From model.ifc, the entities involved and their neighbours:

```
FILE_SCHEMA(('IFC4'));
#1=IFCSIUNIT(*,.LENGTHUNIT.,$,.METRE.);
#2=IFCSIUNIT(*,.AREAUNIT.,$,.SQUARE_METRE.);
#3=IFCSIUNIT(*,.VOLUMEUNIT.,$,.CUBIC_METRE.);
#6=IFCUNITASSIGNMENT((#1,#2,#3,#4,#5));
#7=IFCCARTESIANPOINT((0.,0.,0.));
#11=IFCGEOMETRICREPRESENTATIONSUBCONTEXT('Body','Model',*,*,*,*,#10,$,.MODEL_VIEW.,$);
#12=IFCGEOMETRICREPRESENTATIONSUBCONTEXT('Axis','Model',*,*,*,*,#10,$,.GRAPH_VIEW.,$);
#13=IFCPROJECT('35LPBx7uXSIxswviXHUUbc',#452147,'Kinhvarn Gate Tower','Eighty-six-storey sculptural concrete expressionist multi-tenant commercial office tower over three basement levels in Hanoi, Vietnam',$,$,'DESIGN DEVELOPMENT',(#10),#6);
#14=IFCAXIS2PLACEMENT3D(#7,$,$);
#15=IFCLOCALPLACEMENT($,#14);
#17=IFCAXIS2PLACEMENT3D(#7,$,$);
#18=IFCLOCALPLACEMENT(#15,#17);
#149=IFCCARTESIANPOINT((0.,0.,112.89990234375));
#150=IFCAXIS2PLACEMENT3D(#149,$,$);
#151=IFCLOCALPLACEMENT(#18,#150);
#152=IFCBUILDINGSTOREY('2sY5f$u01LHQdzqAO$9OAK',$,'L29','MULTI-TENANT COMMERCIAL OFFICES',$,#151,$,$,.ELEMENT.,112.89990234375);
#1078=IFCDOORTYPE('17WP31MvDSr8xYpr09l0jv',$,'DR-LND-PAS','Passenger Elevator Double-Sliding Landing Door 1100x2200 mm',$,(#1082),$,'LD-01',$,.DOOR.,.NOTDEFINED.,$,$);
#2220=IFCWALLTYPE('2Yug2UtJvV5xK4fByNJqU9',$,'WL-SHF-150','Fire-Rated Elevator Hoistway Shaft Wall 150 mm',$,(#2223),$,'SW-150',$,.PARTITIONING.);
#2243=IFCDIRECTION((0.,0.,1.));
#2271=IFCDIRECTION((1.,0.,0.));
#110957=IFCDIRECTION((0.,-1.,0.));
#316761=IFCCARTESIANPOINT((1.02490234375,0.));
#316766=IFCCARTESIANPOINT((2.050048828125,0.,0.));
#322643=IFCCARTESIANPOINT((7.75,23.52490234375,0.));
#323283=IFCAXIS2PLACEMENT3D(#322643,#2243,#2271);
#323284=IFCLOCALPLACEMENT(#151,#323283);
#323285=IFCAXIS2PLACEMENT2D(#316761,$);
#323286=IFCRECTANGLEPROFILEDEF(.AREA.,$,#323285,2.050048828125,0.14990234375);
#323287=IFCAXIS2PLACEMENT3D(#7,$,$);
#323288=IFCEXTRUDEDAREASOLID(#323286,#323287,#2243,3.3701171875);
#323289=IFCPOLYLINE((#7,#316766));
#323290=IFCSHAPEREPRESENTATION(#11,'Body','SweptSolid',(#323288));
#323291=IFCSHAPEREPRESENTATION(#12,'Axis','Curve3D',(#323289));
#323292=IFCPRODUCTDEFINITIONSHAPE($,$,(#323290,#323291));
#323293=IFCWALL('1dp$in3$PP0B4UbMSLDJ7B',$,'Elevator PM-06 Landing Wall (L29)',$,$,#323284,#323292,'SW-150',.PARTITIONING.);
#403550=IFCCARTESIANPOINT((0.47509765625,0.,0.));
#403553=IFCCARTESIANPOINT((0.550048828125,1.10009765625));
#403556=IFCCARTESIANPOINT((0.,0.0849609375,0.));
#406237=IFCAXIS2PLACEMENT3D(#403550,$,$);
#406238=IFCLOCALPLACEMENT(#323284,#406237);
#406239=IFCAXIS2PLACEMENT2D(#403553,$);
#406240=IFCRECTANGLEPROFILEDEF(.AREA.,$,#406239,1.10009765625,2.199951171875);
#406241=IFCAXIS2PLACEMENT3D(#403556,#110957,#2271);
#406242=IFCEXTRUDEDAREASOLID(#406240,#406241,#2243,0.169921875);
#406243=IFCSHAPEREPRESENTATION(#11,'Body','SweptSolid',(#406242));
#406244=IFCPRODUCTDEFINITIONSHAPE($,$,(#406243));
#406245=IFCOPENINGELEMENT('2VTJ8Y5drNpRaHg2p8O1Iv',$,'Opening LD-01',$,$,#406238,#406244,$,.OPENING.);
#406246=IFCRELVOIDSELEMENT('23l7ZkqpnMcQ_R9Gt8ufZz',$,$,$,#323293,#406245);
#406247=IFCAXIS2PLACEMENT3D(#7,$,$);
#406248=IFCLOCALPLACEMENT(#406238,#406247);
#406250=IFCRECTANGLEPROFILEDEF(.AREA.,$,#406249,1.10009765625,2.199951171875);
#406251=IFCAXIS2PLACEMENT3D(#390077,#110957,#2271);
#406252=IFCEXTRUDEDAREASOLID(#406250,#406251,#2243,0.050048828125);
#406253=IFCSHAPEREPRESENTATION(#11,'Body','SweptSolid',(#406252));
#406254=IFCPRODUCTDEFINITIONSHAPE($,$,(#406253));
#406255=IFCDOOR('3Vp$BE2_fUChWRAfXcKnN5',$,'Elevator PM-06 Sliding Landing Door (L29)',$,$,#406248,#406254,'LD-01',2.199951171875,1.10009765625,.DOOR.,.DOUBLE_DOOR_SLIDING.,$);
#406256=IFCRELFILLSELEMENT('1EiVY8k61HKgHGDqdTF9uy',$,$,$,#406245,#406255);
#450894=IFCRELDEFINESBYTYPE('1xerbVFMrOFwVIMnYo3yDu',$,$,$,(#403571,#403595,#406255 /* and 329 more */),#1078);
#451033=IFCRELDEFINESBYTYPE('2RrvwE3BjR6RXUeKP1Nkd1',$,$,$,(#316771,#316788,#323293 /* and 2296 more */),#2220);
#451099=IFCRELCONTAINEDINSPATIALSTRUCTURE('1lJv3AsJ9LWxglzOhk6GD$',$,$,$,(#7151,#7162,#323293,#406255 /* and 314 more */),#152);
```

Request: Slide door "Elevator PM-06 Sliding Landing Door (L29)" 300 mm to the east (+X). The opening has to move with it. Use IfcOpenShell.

```python
import ifcopenshell
import ifcopenshell.api.geometry
import ifcopenshell.util.placement
import ifcopenshell.util.unit

model = ifcopenshell.open("model.ifc")
unit_scale = ifcopenshell.util.unit.calculate_unit_scale(model)

door = model.by_guid("3Vp$BE2_fUChWRAfXcKnN5")
opening = door.FillsVoids[0].RelatingOpeningElement
wall = opening.VoidsElements[0].RelatingBuildingElement

wall_matrix = ifcopenshell.util.placement.get_local_placement(wall.ObjectPlacement)
shift = wall_matrix[:3, 0] * 0.3 / unit_scale
before = ifcopenshell.util.placement.get_local_placement(door.ObjectPlacement)[:3, 3].copy()

# The door is placed relative to its opening, so it follows when the opening moves.
matrix = ifcopenshell.util.placement.get_local_placement(opening.ObjectPlacement)
matrix[:3, 3] += shift
ifcopenshell.api.geometry.edit_object_placement(
    model, product=opening, matrix=matrix, is_si=False, should_transform_children=True
)

after = ifcopenshell.util.placement.get_local_placement(door.ObjectPlacement)[:3, 3]
print("door moved by", (after - before).round(3) + 0.0)

model.write("model_v2.ifc")
```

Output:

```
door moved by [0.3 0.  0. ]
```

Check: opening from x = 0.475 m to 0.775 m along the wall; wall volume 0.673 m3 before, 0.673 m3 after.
